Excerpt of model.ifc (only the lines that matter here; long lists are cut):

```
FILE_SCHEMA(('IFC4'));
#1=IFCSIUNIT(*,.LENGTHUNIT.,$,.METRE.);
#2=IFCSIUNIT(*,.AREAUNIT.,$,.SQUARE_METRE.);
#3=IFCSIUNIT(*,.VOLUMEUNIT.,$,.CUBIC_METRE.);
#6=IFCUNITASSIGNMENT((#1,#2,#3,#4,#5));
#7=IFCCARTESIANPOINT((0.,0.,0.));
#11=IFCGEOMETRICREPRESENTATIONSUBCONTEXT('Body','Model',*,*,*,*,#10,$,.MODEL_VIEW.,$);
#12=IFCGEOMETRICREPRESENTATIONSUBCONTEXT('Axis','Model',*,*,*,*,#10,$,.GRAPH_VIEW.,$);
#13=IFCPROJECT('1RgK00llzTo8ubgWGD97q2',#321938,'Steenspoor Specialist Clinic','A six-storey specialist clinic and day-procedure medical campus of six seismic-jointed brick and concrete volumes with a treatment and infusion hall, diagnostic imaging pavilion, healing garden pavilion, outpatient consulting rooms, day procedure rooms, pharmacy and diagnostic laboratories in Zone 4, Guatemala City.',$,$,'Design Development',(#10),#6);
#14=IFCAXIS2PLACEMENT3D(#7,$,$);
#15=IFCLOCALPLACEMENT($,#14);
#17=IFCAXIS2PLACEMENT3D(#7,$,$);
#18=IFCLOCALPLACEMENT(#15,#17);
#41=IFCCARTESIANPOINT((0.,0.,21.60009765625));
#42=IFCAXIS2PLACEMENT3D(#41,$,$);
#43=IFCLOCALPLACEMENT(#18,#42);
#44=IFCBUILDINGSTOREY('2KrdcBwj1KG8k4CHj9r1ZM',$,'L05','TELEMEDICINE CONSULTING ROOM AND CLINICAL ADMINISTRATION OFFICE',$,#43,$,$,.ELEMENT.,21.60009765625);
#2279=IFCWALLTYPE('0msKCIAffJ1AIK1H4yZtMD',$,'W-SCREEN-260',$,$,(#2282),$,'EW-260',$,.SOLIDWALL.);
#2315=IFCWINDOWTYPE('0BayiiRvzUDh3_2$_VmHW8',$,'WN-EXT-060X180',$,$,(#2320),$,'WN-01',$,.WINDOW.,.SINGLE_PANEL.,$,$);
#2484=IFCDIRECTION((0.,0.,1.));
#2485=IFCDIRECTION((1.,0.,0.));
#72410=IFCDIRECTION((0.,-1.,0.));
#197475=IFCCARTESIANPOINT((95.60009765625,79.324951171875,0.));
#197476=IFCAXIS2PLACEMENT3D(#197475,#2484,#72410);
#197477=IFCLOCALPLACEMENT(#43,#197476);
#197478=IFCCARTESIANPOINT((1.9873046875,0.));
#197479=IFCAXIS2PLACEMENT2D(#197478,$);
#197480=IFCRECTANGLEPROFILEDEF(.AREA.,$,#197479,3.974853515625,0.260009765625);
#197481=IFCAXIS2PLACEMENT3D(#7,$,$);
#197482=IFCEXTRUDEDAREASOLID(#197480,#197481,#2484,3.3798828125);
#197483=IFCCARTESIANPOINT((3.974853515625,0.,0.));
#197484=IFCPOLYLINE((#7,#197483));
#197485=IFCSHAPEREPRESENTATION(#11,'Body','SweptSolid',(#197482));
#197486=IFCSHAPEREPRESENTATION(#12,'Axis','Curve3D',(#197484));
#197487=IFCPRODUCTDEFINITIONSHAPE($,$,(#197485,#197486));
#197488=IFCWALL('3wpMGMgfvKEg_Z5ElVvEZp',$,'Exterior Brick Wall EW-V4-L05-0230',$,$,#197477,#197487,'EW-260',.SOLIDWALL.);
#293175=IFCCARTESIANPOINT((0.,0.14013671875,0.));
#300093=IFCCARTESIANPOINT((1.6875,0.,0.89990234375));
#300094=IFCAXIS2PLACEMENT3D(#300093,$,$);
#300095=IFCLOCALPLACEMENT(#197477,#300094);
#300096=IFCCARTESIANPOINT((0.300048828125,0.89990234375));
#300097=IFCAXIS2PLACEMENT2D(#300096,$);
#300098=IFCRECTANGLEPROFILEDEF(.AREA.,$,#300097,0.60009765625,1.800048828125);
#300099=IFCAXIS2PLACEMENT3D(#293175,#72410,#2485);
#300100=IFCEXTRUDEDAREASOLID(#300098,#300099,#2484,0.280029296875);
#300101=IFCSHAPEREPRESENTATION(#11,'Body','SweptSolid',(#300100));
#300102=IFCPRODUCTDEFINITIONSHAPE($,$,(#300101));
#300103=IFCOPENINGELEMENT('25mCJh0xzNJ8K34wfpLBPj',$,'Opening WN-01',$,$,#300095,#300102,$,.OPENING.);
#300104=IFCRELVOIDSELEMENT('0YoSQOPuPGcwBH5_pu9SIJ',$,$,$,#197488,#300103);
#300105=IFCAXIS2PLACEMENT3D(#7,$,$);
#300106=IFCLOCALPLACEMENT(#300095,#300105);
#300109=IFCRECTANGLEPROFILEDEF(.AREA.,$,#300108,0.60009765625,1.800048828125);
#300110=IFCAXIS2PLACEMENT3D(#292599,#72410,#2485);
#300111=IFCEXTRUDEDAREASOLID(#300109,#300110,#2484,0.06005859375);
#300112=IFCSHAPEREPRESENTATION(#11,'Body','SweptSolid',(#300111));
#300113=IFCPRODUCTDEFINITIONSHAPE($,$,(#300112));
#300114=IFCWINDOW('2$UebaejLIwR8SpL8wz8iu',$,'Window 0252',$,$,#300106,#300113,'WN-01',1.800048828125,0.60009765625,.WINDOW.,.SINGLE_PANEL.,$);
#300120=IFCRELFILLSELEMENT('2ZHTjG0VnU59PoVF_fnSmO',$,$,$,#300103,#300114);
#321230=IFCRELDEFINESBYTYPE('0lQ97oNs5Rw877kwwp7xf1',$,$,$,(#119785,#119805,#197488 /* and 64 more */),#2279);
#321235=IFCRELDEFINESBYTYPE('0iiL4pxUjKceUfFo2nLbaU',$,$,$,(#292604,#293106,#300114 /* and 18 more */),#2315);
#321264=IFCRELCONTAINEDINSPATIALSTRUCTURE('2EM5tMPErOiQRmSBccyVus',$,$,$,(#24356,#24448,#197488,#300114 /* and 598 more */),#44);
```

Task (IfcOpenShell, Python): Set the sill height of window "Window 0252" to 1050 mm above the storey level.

```python
import numpy as np
import ifcopenshell
import ifcopenshell.api.geometry
import ifcopenshell.geom
import ifcopenshell.util.element
import ifcopenshell.util.placement
import ifcopenshell.util.shape
import ifcopenshell.util.unit

model = ifcopenshell.open("model.ifc")
unit_scale = ifcopenshell.util.unit.calculate_unit_scale(model)

window = model.by_guid("2$UebaejLIwR8SpL8wz8iu")
opening = window.FillsVoids[0].RelatingOpeningElement
storey = ifcopenshell.util.element.get_container(window, ifc_class="IfcBuildingStorey")
level = ifcopenshell.util.placement.get_local_placement(storey.ObjectPlacement)[2, 3]

# The opening's origin need not be at the sill, so measure its lowest point.
shape = ifcopenshell.geom.create_shape(ifcopenshell.geom.settings(), opening)
bottom = ifcopenshell.util.shape.get_shape_bottom_elevation(shape, shape.geometry) / unit_scale
dz = level + 1.05 / unit_scale - bottom

shift = np.array([0.0, 0.0, dz])
# The window is placed relative to its opening, so it follows when the opening moves.
matrix = ifcopenshell.util.placement.get_local_placement(opening.ObjectPlacement)
matrix[:3, 3] += shift
ifcopenshell.api.geometry.edit_object_placement(
    model, product=opening, matrix=matrix, is_si=False, should_transform_children=True
)

print(f"moved by {dz * unit_scale:+.3f} m")

model.write("model_updated.ifc")
```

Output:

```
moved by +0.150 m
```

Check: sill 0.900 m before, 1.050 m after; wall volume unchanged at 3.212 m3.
